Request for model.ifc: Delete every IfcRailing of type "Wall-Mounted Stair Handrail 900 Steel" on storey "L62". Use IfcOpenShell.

First a look at what the model holds.

```python
import ifcopenshell
import ifcopenshell.util.element

model = ifcopenshell.open("model.ifc")
print(model.schema)
storey = next(s for s in model.by_type("IfcBuildingStorey") if s.Name == "L62")
railings = [e for e in ifcopenshell.util.element.get_decomposition(storey) if e.is_a("IfcRailing")]
seen = {}
for e in railings:
    element_type = ifcopenshell.util.element.get_type(e)
    name = element_type.Name if element_type not in (None, e) else None
    seen[name] = seen.get(name, 0) + 1
for name, count in sorted(seen.items(), key=str):
    print(count, "x", name)
```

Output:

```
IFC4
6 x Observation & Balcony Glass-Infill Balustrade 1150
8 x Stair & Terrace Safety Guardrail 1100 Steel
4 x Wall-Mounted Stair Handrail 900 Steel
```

```python
import ifcopenshell
import ifcopenshell.api.root
import ifcopenshell.util.element

model = ifcopenshell.open("model.ifc")

storey = next(s for s in model.by_type("IfcBuildingStorey") if s.Name == "L62")
railings = [e for e in ifcopenshell.util.element.get_decomposition(storey) if e.is_a("IfcRailing")]
targets = [e for e in railings if (t := ifcopenshell.util.element.get_type(e)) not in (None, e) and t.Name == "Wall-Mounted Stair Handrail 900 Steel"]

for e in targets:
    ifcopenshell.api.root.remove_product(model, product=e)
print(len(targets), "removed")

model.write("model_rev.ifc")
```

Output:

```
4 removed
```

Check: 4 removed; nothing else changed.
